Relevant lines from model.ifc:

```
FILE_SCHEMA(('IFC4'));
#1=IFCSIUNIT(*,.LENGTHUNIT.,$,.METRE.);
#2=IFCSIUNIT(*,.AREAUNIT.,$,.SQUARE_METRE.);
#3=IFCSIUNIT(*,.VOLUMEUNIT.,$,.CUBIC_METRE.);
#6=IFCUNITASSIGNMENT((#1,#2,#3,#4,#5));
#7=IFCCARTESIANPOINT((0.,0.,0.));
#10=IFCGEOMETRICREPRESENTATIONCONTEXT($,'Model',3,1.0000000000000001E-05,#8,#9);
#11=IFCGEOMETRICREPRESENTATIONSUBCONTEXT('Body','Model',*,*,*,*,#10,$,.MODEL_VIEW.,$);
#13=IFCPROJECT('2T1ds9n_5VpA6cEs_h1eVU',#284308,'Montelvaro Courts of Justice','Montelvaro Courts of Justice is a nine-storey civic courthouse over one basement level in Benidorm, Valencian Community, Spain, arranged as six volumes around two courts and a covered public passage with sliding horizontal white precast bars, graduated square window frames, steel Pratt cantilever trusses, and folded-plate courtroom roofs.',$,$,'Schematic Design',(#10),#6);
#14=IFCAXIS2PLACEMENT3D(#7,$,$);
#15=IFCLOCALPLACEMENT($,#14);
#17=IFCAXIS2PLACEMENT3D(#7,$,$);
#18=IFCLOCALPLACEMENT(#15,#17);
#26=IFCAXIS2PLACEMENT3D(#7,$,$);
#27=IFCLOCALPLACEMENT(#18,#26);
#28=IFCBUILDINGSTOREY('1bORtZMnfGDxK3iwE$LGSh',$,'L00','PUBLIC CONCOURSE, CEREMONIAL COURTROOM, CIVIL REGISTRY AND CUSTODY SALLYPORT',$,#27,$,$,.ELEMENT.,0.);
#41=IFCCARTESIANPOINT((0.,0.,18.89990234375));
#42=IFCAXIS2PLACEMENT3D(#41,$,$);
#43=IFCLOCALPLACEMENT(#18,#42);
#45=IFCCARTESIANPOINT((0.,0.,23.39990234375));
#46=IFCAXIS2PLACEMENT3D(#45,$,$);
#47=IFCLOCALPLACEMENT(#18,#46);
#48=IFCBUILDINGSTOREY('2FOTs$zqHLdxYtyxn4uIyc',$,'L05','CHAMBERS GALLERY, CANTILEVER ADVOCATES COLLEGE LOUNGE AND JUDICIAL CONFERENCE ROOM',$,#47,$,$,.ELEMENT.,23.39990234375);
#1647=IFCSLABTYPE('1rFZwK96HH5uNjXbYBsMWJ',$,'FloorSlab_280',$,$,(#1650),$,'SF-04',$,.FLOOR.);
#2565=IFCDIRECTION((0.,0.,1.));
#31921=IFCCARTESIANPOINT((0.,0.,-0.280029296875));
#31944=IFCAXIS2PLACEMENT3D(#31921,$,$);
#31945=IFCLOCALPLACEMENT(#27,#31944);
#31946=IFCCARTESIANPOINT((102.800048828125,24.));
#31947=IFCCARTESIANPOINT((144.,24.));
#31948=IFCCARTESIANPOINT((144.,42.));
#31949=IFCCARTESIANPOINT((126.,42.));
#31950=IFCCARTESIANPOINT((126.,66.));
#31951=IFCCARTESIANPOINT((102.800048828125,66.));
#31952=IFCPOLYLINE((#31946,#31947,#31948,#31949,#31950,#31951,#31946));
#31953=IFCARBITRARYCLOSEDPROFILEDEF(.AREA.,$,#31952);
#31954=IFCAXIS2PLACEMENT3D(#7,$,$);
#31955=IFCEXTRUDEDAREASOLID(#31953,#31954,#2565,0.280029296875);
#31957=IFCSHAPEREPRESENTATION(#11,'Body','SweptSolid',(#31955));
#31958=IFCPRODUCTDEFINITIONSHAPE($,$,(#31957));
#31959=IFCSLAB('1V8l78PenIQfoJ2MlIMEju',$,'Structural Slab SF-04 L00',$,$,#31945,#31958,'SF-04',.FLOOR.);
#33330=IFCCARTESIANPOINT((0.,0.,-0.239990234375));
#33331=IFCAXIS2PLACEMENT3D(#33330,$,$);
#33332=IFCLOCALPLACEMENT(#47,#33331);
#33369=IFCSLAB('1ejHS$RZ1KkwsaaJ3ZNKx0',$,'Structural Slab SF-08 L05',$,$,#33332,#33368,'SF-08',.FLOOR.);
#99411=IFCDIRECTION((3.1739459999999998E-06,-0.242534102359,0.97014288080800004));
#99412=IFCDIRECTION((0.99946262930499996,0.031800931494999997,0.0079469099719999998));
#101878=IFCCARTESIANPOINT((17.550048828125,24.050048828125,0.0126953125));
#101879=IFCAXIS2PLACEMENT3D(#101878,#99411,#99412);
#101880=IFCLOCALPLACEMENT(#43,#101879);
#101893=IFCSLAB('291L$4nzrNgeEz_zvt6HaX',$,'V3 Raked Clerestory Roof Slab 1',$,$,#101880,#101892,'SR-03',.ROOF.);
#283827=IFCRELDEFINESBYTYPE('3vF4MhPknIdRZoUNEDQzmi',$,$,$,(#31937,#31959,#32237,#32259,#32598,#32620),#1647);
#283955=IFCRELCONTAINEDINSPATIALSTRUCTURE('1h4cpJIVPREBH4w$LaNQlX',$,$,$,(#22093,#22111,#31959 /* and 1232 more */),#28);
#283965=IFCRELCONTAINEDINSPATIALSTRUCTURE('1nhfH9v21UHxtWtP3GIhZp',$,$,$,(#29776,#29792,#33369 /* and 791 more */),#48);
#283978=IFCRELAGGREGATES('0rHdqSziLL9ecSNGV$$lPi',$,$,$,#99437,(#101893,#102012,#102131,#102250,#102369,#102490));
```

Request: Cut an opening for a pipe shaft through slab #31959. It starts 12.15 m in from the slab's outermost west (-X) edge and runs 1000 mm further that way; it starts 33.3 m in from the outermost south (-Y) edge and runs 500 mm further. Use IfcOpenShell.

```python
import numpy as np
import ifcopenshell
import ifcopenshell.api.feature
import ifcopenshell.api.geometry
import ifcopenshell.api.root
import ifcopenshell.geom
import ifcopenshell.util.placement
import ifcopenshell.util.representation
import ifcopenshell.util.shape
import ifcopenshell.util.unit

model = ifcopenshell.open("model.ifc")
unit_scale = ifcopenshell.util.unit.calculate_unit_scale(model)
settings = ifcopenshell.geom.settings()


def volume(element):
    """Net volume in cubic metres, openings subtracted."""
    shape = ifcopenshell.geom.create_shape(settings, element)
    return ifcopenshell.util.shape.get_volume(shape.geometry)


slab = model.by_id(31959)
before = volume(slab)

# Extent in the slab's own axes, in metres. The edges named are its -X and -Y sides.
slab_shape = ifcopenshell.geom.create_shape(settings, slab)
vertices = ifcopenshell.util.shape.get_vertices(slab_shape.geometry)
x_min, y_min, bottom = vertices.min(axis=0)
top = vertices[:, 2].max()

opening = ifcopenshell.api.root.create_entity(model, ifc_class="IfcOpeningElement", name="Pipe shaft opening", predefined_type="OPENING")
context = ifcopenshell.util.representation.get_context(model, "Model", "Body", "MODEL_VIEW")
width, depth = 1, 0.5
outline = [(0.0, 0.0), (width, 0.0), (width, depth), (0.0, depth), (0.0, 0.0)]
# Overshoot both faces by 50 mm so the cut is clean.
shape = ifcopenshell.api.geometry.add_slab_representation(
    model, context=context, depth=top - bottom + 0.1, polyline=outline
)
ifcopenshell.api.geometry.assign_representation(model, product=opening, representation=shape)

matrix = ifcopenshell.util.placement.get_local_placement(slab.ObjectPlacement)
matrix[:, 3] = matrix @ np.append(np.array([x_min + 12.15, y_min + 33.3, bottom - 0.05]) / unit_scale, 1.0)
ifcopenshell.api.geometry.edit_object_placement(model, product=opening, matrix=matrix, is_si=False)
ifcopenshell.api.feature.add_feature(model, feature=opening, element=slab)

after = volume(slab)

print(f"slab volume {before:.3f} -> {after:.3f} m3")

model.write("model-out.ifc")
```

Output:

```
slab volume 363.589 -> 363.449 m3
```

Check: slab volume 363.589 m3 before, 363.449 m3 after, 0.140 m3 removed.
